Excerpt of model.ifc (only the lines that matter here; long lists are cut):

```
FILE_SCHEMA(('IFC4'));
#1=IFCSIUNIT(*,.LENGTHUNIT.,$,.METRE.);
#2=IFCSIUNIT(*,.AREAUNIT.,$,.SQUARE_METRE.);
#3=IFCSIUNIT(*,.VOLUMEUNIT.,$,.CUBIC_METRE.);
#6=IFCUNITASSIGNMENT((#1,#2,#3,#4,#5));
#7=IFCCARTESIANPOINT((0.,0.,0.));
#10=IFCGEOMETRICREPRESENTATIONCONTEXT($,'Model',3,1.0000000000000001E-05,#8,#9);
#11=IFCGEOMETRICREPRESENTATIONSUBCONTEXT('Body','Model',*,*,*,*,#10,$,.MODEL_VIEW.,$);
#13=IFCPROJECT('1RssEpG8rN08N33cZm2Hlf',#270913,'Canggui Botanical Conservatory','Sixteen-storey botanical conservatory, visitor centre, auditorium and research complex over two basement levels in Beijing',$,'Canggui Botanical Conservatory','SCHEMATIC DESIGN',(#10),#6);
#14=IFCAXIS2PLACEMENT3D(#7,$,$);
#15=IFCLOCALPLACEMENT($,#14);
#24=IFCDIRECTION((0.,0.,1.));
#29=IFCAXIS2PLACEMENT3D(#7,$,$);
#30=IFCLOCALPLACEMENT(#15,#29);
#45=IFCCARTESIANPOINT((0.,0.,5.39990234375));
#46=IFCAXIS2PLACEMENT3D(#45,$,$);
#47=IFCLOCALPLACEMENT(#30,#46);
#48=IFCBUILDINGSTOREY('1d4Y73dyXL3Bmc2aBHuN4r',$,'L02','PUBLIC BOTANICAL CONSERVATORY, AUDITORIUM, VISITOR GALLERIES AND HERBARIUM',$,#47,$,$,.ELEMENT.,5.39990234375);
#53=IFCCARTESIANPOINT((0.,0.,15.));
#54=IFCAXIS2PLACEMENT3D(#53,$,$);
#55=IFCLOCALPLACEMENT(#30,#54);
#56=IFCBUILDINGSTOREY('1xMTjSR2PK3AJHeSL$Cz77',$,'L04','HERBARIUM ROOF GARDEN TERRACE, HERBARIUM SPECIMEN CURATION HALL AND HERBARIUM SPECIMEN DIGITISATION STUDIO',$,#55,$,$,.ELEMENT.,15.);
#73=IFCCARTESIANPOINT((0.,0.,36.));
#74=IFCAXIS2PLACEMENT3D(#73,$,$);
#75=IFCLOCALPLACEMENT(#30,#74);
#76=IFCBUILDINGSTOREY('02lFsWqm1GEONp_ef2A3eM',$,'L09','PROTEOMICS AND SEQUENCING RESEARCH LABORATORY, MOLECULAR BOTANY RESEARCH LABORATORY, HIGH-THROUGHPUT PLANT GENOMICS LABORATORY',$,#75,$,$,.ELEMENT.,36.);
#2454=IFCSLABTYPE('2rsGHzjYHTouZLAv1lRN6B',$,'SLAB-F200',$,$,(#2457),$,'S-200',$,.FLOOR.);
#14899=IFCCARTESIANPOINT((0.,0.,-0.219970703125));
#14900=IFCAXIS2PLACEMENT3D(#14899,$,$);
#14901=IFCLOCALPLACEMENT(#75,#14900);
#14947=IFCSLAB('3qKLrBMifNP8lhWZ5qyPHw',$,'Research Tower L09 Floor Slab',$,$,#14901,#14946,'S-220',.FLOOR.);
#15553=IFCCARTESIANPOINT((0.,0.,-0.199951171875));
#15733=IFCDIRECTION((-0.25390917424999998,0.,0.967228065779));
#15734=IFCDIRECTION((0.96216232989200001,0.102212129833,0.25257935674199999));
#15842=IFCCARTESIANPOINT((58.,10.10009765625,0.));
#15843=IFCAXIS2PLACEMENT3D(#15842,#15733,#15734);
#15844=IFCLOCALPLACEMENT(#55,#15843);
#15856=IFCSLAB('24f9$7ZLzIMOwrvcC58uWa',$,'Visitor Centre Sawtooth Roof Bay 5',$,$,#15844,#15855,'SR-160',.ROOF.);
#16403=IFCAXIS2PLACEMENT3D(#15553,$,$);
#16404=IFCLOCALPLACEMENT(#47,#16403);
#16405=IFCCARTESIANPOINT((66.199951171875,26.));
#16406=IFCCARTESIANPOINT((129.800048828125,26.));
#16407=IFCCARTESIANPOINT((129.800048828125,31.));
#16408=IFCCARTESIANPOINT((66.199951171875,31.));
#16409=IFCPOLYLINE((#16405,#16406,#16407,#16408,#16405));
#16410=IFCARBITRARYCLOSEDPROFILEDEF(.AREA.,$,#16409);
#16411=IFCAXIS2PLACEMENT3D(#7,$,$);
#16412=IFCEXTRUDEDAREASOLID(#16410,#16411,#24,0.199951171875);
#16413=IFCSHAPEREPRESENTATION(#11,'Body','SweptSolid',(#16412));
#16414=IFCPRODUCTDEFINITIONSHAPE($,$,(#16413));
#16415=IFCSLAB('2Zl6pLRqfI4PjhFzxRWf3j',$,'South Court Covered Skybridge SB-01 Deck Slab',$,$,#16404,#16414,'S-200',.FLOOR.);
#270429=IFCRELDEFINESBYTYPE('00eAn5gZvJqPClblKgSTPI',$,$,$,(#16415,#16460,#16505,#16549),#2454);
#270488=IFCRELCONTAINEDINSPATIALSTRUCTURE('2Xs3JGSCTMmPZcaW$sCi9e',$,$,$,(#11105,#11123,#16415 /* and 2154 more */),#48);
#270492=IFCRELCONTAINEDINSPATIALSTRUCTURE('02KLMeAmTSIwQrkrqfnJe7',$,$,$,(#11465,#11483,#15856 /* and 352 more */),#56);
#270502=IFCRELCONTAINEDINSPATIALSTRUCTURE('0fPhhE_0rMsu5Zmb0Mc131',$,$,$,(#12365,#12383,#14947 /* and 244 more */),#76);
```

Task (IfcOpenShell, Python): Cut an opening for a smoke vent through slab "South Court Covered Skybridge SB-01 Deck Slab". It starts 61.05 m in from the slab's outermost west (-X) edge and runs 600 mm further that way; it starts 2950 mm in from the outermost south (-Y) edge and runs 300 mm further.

```python
import numpy as np
import ifcopenshell
import ifcopenshell.api.feature
import ifcopenshell.api.geometry
import ifcopenshell.api.root
import ifcopenshell.geom
import ifcopenshell.util.placement
import ifcopenshell.util.representation
import ifcopenshell.util.shape
import ifcopenshell.util.unit

model = ifcopenshell.open("model.ifc")
unit_scale = ifcopenshell.util.unit.calculate_unit_scale(model)
settings = ifcopenshell.geom.settings()


def volume(element):
    """Net volume in cubic metres, openings subtracted."""
    shape = ifcopenshell.geom.create_shape(settings, element)
    return ifcopenshell.util.shape.get_volume(shape.geometry)


slab = model.by_id(16415)
before = volume(slab)

# Extent in the slab's own axes, in metres. The edges named are its -X and -Y sides.
slab_shape = ifcopenshell.geom.create_shape(settings, slab)
vertices = ifcopenshell.util.shape.get_vertices(slab_shape.geometry)
x_min, y_min, bottom = vertices.min(axis=0)
top = vertices[:, 2].max()

opening = ifcopenshell.api.root.create_entity(model, ifc_class="IfcOpeningElement", name="Smoke vent opening", predefined_type="OPENING")
context = ifcopenshell.util.representation.get_context(model, "Model", "Body", "MODEL_VIEW")
width, depth = 0.6, 0.3
outline = [(0.0, 0.0), (width, 0.0), (width, depth), (0.0, depth), (0.0, 0.0)]
# Overshoot both faces by 50 mm so the cut is clean.
shape = ifcopenshell.api.geometry.add_slab_representation(
    model, context=context, depth=top - bottom + 0.1, polyline=outline
)
ifcopenshell.api.geometry.assign_representation(model, product=opening, representation=shape)

matrix = ifcopenshell.util.placement.get_local_placement(slab.ObjectPlacement)
matrix[:, 3] = matrix @ np.append(np.array([x_min + 61.05, y_min + 2.95, bottom - 0.05]) / unit_scale, 1.0)
ifcopenshell.api.geometry.edit_object_placement(model, product=opening, matrix=matrix, is_si=False)
ifcopenshell.api.feature.add_feature(model, feature=opening, element=slab)

after = volume(slab)

print(f"slab volume {before:.3f} -> {after:.3f} m3")

model.write("model_rev.ifc")
```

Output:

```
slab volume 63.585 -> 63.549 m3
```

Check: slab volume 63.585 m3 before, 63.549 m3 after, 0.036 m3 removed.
